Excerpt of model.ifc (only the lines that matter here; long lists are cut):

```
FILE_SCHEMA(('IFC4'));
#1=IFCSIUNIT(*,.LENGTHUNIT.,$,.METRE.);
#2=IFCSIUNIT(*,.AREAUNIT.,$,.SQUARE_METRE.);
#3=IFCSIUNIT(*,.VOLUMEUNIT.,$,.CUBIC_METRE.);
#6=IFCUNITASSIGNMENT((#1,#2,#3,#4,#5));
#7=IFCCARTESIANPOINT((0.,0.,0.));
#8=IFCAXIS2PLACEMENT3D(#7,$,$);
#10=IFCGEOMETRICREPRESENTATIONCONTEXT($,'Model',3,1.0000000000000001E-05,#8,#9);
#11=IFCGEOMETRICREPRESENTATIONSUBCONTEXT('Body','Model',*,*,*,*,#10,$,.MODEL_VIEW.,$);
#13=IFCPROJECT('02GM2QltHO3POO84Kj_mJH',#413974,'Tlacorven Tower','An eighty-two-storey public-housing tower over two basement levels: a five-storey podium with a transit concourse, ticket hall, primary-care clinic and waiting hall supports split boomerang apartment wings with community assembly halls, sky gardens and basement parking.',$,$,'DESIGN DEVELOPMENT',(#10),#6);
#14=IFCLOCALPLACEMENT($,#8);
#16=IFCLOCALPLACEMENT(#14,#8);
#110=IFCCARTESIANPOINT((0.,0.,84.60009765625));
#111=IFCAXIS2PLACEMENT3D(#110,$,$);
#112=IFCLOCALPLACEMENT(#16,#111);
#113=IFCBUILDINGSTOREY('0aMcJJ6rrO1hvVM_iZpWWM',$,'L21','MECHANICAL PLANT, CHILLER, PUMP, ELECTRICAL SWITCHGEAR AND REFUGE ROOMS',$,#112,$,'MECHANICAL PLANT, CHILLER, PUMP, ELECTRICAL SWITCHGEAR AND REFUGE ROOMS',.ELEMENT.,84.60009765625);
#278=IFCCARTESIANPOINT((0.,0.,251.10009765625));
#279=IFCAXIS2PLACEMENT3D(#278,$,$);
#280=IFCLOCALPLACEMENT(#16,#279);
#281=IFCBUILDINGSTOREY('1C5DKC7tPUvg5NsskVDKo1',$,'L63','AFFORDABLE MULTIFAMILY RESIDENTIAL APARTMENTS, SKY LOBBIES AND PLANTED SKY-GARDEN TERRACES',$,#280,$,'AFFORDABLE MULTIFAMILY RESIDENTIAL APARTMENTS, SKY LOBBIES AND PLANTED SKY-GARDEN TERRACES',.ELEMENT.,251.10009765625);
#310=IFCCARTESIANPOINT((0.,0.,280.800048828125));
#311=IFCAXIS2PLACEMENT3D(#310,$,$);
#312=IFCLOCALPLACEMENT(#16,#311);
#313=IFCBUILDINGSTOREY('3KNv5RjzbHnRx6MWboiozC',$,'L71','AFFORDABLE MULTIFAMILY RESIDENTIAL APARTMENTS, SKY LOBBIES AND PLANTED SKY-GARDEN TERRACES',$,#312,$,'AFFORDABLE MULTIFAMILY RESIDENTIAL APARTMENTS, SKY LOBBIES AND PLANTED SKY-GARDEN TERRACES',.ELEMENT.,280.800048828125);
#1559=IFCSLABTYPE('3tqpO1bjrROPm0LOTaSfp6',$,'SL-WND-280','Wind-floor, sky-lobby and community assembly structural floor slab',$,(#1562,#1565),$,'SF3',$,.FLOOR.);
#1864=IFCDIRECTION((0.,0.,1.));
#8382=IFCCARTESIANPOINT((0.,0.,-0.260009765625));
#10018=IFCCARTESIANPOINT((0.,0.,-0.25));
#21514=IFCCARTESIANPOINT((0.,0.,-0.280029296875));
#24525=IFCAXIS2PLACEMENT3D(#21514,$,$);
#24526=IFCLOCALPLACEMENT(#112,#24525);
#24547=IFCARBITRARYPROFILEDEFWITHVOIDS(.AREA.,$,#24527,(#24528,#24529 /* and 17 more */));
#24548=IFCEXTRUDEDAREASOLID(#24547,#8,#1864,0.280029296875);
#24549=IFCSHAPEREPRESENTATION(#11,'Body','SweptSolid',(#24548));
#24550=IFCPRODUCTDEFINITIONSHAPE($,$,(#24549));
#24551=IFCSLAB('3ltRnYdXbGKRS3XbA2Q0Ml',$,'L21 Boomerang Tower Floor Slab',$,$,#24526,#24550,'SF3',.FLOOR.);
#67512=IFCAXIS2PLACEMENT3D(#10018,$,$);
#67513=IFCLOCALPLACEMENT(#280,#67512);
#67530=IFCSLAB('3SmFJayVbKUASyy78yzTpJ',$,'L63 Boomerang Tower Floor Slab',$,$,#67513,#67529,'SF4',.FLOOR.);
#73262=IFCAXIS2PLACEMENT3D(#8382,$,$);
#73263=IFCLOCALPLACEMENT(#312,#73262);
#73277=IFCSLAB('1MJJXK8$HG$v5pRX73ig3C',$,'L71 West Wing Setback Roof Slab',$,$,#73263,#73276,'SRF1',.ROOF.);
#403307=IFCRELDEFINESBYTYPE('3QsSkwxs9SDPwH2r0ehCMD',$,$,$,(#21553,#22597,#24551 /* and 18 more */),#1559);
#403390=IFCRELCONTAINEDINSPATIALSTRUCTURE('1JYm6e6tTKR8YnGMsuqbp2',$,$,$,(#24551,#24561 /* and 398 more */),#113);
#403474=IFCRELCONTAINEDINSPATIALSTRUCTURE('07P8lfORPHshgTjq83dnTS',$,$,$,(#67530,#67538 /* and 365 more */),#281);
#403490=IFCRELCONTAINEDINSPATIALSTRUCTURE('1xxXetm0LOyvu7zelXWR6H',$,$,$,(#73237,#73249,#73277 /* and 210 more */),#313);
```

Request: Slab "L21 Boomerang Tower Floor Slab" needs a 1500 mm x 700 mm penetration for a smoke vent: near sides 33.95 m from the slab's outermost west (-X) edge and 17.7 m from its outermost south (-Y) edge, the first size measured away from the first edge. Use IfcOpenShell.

```python
import numpy as np
import ifcopenshell
import ifcopenshell.api.feature
import ifcopenshell.api.geometry
import ifcopenshell.api.root
import ifcopenshell.geom
import ifcopenshell.util.placement
import ifcopenshell.util.representation
import ifcopenshell.util.shape
import ifcopenshell.util.unit

model = ifcopenshell.open("model.ifc")
unit_scale = ifcopenshell.util.unit.calculate_unit_scale(model)
settings = ifcopenshell.geom.settings()


def volume(element):
    """Net volume in cubic metres, openings subtracted."""
    shape = ifcopenshell.geom.create_shape(settings, element)
    return ifcopenshell.util.shape.get_volume(shape.geometry)


slab = model.by_guid("3ltRnYdXbGKRS3XbA2Q0Ml")
before = volume(slab)

# Extent in the slab's own axes, in metres. The edges named are its -X and -Y sides.
slab_shape = ifcopenshell.geom.create_shape(settings, slab)
vertices = ifcopenshell.util.shape.get_vertices(slab_shape.geometry)
x_min, y_min, bottom = vertices.min(axis=0)
top = vertices[:, 2].max()

opening = ifcopenshell.api.root.create_entity(model, ifc_class="IfcOpeningElement", name="Smoke vent opening", predefined_type="OPENING")
context = ifcopenshell.util.representation.get_context(model, "Model", "Body", "MODEL_VIEW")
width, depth = 1.5, 0.7
outline = [(0.0, 0.0), (width, 0.0), (width, depth), (0.0, depth), (0.0, 0.0)]
# Overshoot both faces by 50 mm so the cut is clean.
shape = ifcopenshell.api.geometry.add_slab_representation(
    model, context=context, depth=top - bottom + 0.1, polyline=outline
)
ifcopenshell.api.geometry.assign_representation(model, product=opening, representation=shape)

matrix = ifcopenshell.util.placement.get_local_placement(slab.ObjectPlacement)
matrix[:, 3] = matrix @ np.append(np.array([x_min + 33.95, y_min + 17.7, bottom - 0.05]) / unit_scale, 1.0)
ifcopenshell.api.geometry.edit_object_placement(model, product=opening, matrix=matrix, is_si=False)
ifcopenshell.api.feature.add_feature(model, feature=opening, element=slab)

after = volume(slab)

print(f"slab volume {before:.3f} -> {after:.3f} m3")

model.write("model_edited.ifc")
```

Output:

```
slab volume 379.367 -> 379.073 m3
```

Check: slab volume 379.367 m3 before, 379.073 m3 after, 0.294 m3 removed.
